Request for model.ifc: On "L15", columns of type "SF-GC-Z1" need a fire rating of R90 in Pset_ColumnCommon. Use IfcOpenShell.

First a look at what the model holds.

```python
import ifcopenshell
import ifcopenshell.util.element

model = ifcopenshell.open("model.ifc")
print(model.schema)
storey = next(s for s in model.by_type("IfcBuildingStorey") if s.Name == "L15")
columns = [e for e in ifcopenshell.util.element.get_decomposition(storey) if e.is_a("IfcColumn")]
seen = {}
for e in columns:
    element_type = ifcopenshell.util.element.get_type(e)
    key = (element_type.Name if element_type != e and element_type else None, ifcopenshell.util.element.get_pset(e, "Pset_ColumnCommon", "FireRating"))
    seen[key] = seen.get(key, 0) + 1
for (name, value), count in sorted(seen.items(), key=str):
    print(count, "x", name, "|", value)
```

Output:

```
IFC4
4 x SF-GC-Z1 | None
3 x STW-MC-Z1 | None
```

```python
import ifcopenshell
import ifcopenshell.api.pset
import ifcopenshell.util.element

model = ifcopenshell.open("model.ifc")

storey = next(s for s in model.by_type("IfcBuildingStorey") if s.Name == "L15")
columns = [e for e in ifcopenshell.util.element.get_decomposition(storey) if e.is_a("IfcColumn")]

count = 0
for e in columns:
    element_type = ifcopenshell.util.element.get_type(e)
    if element_type in (None, e) or element_type.Name != "SF-GC-Z1":
        continue
    found = ifcopenshell.util.element.get_pset(e, "Pset_ColumnCommon", should_inherit=False)
    if found:
        pset = model.by_id(found["id"])
        if len(ifcopenshell.util.element.get_elements_by_pset(pset)) > 1:
            pset = ifcopenshell.api.pset.unshare_pset(model, products=[e], pset=pset)[0]
    else:
        pset = ifcopenshell.api.pset.add_pset(model, product=e, name="Pset_ColumnCommon")
    ifcopenshell.api.pset.edit_pset(model, pset=pset, properties={"FireRating": "R90"})
    count += 1

print(count, "columns updated")

model.write("model_edited.ifc")
```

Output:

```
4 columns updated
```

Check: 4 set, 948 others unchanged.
